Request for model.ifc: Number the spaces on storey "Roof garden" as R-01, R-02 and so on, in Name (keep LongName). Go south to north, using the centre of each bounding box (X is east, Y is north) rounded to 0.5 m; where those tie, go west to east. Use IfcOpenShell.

First a look at what the model holds.

```python
import ifcopenshell
import ifcopenshell.util.element
import ifcopenshell.util.placement

model = ifcopenshell.open("model.ifc")
print(model.schema)
storey = next(s for s in model.by_type("IfcBuildingStorey") if s.Name == "Roof garden")
spaces = [e for e in ifcopenshell.util.element.get_decomposition(storey) if e.is_a("IfcSpace")]
for e in sorted(spaces, key=lambda e: e.id()):
    origin = ifcopenshell.util.placement.get_local_placement(e.ObjectPlacement)[:3, 3]
    print(e.id(), e.Name, e.LongName, origin.round(2) + 0.0, sep=" | ")
```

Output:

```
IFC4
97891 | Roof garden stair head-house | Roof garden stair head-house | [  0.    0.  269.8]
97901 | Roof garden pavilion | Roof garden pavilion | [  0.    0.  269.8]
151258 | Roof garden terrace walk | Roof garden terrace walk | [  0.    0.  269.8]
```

```python
import ifcopenshell
import ifcopenshell.geom
import ifcopenshell.util.element
import ifcopenshell.util.shape

model = ifcopenshell.open("model.ifc")
settings = ifcopenshell.geom.settings()
settings.set("use-world-coords", True)


def centre(element):
    shape = ifcopenshell.geom.create_shape(settings, element)
    return ifcopenshell.util.shape.get_bbox_centroid(shape.geometry)


storey = next(s for s in model.by_type("IfcBuildingStorey") if s.Name == "Roof garden")
spaces = [e for e in ifcopenshell.util.element.get_decomposition(storey) if e.is_a("IfcSpace")]

# Insertion points can sit at a corner or the storey origin, so sort by the geometry (in metres).
centres = {e: centre(e) for e in spaces}
spaces.sort(key=lambda e: (round(centres[e][1] / 0.5), centres[e][0]))

for i, e in enumerate(spaces, start=1):
    number = f"R-{i:02d}"
    e.Name = number
    print(e.id(), number)

model.write("model-out.ifc")
```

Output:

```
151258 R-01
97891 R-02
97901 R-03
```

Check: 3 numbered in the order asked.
